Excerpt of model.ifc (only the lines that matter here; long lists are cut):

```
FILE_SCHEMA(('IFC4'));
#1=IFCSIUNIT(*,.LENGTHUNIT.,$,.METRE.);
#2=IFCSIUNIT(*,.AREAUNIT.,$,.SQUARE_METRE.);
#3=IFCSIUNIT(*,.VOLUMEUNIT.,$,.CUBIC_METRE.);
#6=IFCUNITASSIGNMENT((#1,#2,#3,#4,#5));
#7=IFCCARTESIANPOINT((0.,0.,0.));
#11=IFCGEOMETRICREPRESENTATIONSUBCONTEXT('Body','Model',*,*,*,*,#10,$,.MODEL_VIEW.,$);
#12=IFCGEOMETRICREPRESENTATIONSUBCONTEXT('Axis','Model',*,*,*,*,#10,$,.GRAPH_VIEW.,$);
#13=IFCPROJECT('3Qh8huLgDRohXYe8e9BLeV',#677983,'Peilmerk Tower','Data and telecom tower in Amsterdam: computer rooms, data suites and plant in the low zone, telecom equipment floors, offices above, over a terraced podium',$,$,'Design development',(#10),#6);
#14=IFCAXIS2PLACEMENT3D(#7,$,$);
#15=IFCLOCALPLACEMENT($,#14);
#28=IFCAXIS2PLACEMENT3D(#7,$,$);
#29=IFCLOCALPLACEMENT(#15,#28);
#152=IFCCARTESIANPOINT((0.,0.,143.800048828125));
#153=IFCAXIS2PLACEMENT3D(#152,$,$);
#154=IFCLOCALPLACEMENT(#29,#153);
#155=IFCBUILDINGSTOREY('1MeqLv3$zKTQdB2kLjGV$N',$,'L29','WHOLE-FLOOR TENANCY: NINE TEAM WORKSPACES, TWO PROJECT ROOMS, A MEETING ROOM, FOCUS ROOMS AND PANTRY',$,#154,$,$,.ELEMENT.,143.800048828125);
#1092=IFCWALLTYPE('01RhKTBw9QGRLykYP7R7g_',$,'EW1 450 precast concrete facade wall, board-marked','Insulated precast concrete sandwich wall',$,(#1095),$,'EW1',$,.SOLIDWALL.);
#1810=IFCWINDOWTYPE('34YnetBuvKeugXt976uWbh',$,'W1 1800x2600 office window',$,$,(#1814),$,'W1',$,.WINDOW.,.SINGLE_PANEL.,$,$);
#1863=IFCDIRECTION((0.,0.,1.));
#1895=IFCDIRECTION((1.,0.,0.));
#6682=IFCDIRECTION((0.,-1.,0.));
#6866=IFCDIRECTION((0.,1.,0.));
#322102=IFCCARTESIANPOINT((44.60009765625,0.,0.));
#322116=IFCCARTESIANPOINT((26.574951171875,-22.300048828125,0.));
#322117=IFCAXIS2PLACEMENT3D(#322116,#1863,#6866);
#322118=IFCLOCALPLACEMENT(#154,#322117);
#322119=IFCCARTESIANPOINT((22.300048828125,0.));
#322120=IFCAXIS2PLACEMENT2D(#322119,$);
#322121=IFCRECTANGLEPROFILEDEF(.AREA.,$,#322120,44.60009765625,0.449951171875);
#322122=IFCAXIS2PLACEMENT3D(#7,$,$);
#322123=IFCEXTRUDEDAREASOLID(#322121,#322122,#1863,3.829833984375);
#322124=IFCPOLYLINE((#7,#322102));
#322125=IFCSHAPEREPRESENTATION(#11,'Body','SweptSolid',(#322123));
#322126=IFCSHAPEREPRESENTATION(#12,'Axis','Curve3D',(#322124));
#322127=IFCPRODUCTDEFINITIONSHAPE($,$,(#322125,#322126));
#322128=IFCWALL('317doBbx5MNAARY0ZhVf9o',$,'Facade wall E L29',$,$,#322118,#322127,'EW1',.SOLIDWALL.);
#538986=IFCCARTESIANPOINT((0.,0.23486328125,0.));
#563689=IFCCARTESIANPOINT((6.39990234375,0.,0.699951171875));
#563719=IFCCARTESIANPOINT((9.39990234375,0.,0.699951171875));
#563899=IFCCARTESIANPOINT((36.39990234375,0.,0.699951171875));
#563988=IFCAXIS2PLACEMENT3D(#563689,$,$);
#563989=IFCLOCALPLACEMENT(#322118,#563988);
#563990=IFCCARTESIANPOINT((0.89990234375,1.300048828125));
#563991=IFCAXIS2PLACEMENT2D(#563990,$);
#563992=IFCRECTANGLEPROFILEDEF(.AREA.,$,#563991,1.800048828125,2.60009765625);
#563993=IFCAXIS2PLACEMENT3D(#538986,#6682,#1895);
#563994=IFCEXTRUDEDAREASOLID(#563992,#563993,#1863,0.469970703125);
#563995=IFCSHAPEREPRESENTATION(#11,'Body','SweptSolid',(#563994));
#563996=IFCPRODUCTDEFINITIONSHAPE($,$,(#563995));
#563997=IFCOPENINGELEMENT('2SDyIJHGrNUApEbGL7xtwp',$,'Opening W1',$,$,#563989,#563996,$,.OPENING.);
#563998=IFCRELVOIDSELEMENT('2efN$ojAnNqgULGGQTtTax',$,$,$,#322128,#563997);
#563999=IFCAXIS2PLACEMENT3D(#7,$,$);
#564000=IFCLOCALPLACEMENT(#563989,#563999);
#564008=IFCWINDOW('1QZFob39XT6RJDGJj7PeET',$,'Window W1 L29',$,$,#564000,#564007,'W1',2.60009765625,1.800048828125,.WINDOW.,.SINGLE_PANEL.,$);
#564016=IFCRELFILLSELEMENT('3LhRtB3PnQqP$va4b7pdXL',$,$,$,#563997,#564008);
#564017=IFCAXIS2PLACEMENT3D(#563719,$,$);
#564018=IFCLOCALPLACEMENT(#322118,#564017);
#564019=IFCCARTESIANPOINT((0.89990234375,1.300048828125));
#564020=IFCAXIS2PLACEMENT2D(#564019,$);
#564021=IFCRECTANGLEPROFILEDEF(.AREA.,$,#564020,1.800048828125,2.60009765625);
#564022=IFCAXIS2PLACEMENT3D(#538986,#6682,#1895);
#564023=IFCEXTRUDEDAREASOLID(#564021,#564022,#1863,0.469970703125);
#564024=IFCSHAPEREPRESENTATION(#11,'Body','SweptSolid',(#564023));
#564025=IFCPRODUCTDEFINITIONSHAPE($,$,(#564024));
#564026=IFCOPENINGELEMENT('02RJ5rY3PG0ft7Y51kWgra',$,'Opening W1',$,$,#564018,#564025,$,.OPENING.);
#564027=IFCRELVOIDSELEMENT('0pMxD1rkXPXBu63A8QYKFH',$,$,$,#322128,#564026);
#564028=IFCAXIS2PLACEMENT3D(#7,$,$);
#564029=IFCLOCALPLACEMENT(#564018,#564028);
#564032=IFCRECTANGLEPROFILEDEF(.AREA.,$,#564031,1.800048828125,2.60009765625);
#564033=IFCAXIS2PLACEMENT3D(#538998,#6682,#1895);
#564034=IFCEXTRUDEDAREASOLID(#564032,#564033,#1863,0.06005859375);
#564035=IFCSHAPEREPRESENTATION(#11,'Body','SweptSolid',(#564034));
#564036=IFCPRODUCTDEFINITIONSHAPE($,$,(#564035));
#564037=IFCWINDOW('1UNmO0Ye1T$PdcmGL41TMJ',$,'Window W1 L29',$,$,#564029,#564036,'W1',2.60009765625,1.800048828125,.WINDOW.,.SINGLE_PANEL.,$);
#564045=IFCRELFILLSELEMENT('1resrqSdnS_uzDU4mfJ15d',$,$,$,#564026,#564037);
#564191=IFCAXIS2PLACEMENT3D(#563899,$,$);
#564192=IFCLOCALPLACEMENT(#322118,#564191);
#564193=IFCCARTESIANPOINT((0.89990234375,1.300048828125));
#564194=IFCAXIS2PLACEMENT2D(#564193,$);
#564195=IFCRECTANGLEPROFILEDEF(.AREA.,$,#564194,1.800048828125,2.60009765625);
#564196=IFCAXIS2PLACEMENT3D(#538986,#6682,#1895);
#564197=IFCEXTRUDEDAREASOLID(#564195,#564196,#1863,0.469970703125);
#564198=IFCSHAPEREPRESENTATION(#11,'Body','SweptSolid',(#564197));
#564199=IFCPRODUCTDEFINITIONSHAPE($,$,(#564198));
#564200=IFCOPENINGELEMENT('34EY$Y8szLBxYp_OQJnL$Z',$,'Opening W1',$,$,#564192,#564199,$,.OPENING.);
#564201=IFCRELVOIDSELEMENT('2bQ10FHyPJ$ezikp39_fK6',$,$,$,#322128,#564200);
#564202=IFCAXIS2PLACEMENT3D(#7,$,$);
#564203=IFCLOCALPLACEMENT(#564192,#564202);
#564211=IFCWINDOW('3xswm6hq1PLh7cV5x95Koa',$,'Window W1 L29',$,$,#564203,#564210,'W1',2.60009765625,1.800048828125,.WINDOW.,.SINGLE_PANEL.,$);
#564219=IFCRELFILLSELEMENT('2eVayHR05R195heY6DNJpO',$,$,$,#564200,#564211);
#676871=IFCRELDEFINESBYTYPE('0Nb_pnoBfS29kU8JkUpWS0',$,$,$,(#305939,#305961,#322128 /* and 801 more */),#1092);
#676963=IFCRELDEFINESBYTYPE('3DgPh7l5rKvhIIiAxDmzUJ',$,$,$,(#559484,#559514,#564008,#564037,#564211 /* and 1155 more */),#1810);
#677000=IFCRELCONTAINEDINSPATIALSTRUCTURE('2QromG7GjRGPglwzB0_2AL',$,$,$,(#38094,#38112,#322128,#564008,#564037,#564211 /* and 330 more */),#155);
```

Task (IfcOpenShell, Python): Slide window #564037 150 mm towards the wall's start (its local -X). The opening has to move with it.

```python
import ifcopenshell
import ifcopenshell.api.geometry
import ifcopenshell.util.placement
import ifcopenshell.util.unit

model = ifcopenshell.open("model.ifc")
unit_scale = ifcopenshell.util.unit.calculate_unit_scale(model)

window = model.by_id(564037)
opening = window.FillsVoids[0].RelatingOpeningElement
wall = opening.VoidsElements[0].RelatingBuildingElement

wall_matrix = ifcopenshell.util.placement.get_local_placement(wall.ObjectPlacement)
shift = wall_matrix[:3, 0] * -0.15 / unit_scale
before = ifcopenshell.util.placement.get_local_placement(window.ObjectPlacement)[:3, 3].copy()

# The window is placed relative to its opening, so it follows when the opening moves.
matrix = ifcopenshell.util.placement.get_local_placement(opening.ObjectPlacement)
matrix[:3, 3] += shift
ifcopenshell.api.geometry.edit_object_placement(
    model, product=opening, matrix=matrix, is_si=False, should_transform_children=True
)

after = ifcopenshell.util.placement.get_local_placement(window.ObjectPlacement)[:3, 3]
print("window moved by", (after - before).round(3) + 0.0)

model.write("model-out.ifc")
```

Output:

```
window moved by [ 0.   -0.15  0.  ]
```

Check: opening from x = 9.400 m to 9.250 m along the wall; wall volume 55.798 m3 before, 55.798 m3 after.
